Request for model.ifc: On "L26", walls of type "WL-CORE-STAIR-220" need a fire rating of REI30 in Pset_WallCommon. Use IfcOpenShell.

First a look at what the model holds.

```python
import ifcopenshell
import ifcopenshell.util.element

model = ifcopenshell.open("model.ifc")
print(model.schema)
storey = next(s for s in model.by_type("IfcBuildingStorey") if s.Name == "L26")
walls = [e for e in ifcopenshell.util.element.get_decomposition(storey) if e.is_a("IfcWall")]
seen = {}
for e in walls:
    element_type = ifcopenshell.util.element.get_type(e)
    key = (element_type.Name if element_type != e and element_type else None, ifcopenshell.util.element.get_pset(e, "Pset_WallCommon", "FireRating"))
    seen[key] = seen.get(key, 0) + 1
for (name, value), count in sorted(seen.items(), key=str):
    print(count, "x", name, "|", value)
```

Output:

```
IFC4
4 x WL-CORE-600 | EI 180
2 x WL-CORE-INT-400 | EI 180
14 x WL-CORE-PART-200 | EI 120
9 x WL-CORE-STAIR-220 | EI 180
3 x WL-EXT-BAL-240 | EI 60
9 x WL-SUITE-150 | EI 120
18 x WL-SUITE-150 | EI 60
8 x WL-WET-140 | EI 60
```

```python
import ifcopenshell
import ifcopenshell.api.pset
import ifcopenshell.util.element

model = ifcopenshell.open("model.ifc")

storey = next(s for s in model.by_type("IfcBuildingStorey") if s.Name == "L26")
walls = [e for e in ifcopenshell.util.element.get_decomposition(storey) if e.is_a("IfcWall")]

count = 0
for e in walls:
    element_type = ifcopenshell.util.element.get_type(e)
    if element_type in (None, e) or element_type.Name != "WL-CORE-STAIR-220":
        continue
    # add_pset returns the element's existing set when there is one.
    pset = ifcopenshell.api.pset.add_pset(model, product=e, name="Pset_WallCommon")
    ifcopenshell.api.pset.edit_pset(model, pset=pset, properties={"FireRating": "REI30"})
    count += 1

print(count, "walls updated")

model.write("model_v2.ifc")
```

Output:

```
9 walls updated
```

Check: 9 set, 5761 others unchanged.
